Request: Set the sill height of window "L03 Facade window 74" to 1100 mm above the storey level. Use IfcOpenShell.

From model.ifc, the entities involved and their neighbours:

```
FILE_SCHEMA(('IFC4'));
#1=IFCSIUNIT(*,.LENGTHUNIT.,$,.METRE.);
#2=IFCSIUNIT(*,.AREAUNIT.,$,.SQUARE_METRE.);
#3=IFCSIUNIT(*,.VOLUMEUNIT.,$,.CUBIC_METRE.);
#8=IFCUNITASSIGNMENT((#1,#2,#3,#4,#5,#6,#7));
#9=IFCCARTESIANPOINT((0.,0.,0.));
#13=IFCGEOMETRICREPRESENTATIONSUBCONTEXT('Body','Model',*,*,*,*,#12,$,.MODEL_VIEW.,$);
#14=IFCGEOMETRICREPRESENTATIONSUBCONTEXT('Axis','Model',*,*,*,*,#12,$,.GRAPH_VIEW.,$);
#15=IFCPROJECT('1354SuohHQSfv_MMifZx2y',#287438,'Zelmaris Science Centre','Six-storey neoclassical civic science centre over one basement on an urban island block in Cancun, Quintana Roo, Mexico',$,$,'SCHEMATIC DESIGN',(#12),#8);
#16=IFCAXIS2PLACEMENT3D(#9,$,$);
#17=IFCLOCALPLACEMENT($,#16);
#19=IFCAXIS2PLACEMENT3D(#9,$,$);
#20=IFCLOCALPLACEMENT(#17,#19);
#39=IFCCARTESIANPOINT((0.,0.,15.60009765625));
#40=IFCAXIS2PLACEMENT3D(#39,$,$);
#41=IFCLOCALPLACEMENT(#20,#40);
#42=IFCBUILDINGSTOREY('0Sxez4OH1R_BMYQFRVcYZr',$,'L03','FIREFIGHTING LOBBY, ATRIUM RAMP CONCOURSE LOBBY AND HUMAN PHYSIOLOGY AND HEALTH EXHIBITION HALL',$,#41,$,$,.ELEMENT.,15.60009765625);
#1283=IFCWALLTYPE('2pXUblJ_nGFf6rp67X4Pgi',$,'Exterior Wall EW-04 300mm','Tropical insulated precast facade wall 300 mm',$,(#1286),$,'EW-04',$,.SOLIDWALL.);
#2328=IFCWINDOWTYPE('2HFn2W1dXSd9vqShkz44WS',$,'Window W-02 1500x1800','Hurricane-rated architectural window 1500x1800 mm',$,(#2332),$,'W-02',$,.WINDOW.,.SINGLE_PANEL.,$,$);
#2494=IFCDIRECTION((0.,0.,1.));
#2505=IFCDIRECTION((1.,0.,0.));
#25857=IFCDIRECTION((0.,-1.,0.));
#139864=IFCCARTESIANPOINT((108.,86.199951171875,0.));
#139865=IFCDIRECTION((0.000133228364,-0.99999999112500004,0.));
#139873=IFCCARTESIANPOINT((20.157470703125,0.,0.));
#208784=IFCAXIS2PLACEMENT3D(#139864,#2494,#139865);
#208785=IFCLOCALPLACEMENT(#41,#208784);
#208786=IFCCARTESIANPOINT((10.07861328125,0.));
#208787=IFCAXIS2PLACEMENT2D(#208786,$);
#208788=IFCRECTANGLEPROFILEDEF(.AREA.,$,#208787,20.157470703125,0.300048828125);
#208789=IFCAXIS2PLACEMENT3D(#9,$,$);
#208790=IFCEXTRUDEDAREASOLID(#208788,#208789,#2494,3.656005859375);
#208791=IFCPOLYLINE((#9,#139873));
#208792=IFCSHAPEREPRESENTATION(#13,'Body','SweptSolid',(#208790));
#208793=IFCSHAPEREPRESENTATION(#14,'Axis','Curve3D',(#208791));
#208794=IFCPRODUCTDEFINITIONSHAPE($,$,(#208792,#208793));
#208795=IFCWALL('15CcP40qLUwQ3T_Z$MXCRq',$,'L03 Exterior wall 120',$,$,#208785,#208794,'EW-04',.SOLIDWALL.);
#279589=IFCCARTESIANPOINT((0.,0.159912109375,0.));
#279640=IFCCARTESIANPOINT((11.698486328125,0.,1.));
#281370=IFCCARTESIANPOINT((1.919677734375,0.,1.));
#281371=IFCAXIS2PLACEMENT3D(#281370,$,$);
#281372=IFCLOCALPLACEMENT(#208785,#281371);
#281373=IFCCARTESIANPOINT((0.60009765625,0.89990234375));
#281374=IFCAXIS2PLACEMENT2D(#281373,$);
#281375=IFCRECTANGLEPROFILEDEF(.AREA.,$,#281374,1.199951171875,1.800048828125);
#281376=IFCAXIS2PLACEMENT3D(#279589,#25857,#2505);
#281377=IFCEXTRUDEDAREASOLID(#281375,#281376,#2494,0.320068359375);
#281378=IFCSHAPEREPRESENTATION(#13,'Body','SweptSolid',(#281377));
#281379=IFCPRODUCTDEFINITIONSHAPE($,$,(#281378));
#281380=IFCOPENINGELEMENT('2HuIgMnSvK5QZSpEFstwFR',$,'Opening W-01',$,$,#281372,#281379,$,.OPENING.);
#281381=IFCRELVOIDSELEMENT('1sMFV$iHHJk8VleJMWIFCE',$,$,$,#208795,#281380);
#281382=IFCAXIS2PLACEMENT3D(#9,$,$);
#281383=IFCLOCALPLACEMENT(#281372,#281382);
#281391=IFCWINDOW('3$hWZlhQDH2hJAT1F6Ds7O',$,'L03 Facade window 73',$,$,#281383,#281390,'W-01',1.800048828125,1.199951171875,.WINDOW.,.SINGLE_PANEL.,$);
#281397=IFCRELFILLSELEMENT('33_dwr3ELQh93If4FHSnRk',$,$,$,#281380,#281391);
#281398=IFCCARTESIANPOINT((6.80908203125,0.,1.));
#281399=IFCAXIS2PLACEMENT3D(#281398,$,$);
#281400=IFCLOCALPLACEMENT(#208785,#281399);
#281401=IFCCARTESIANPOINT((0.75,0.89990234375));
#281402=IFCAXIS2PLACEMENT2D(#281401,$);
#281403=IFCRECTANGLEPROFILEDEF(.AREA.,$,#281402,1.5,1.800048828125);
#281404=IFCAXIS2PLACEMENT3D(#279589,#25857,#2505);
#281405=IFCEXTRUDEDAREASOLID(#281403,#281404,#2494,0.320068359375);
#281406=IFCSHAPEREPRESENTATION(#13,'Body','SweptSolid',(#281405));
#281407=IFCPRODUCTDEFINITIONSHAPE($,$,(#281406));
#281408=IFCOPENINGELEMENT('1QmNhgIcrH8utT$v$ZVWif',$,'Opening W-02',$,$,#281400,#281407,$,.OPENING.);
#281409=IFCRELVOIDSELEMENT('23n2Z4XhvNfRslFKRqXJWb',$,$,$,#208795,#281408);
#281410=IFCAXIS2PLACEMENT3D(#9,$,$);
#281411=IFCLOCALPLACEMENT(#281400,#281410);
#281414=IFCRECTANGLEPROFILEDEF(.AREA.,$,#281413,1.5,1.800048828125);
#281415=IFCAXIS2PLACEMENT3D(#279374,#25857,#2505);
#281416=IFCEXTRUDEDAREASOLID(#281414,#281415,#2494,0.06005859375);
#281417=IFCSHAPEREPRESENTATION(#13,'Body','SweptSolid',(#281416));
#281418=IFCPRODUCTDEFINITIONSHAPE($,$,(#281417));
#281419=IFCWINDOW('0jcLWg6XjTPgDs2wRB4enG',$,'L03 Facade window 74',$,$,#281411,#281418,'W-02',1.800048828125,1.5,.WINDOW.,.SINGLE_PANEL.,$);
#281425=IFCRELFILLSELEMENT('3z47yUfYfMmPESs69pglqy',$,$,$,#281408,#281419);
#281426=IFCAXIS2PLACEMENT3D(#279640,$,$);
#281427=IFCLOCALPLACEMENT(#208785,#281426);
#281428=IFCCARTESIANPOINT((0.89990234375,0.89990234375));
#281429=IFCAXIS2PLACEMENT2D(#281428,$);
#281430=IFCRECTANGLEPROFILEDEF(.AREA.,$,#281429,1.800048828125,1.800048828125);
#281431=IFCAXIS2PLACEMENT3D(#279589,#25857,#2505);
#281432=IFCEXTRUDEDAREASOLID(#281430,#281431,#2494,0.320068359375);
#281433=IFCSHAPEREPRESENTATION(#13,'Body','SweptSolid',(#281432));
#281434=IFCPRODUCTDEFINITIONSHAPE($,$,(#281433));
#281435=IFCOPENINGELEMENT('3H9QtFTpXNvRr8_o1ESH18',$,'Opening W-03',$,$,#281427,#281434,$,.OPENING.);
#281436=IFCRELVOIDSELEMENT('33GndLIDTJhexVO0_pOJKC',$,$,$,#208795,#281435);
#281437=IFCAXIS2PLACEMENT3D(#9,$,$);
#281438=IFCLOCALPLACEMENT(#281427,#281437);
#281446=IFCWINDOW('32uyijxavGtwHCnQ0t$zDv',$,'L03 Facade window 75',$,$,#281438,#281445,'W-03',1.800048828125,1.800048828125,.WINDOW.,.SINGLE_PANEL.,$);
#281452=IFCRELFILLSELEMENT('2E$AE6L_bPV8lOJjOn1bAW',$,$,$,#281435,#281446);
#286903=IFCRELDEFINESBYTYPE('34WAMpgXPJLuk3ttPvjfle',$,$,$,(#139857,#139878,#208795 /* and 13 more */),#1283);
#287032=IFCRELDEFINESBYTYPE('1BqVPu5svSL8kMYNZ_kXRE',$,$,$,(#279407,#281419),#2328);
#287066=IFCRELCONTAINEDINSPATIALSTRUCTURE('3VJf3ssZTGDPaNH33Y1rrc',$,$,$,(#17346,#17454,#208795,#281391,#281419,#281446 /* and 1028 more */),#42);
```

```python
import numpy as np
import ifcopenshell
import ifcopenshell.api.geometry
import ifcopenshell.geom
import ifcopenshell.util.element
import ifcopenshell.util.placement
import ifcopenshell.util.shape
import ifcopenshell.util.unit

model = ifcopenshell.open("model.ifc")
unit_scale = ifcopenshell.util.unit.calculate_unit_scale(model)

window = model.by_guid("0jcLWg6XjTPgDs2wRB4enG")
opening = window.FillsVoids[0].RelatingOpeningElement
storey = ifcopenshell.util.element.get_container(window, ifc_class="IfcBuildingStorey")
level = ifcopenshell.util.placement.get_local_placement(storey.ObjectPlacement)[2, 3]

# The opening's origin need not be at the sill, so measure its lowest point.
shape = ifcopenshell.geom.create_shape(ifcopenshell.geom.settings(), opening)
bottom = ifcopenshell.util.shape.get_shape_bottom_elevation(shape, shape.geometry) / unit_scale
dz = level + 1.1 - bottom

shift = np.array([0.0, 0.0, dz])
# The window is placed relative to its opening, so it follows when the opening moves.
matrix = ifcopenshell.util.placement.get_local_placement(opening.ObjectPlacement)
matrix[:3, 3] += shift
ifcopenshell.api.geometry.edit_object_placement(
    model, product=opening, matrix=matrix, is_si=False, should_transform_children=True
)

print(f"moved by {dz * unit_scale:+.3f} m")

model.write("model_rev.ifc")
```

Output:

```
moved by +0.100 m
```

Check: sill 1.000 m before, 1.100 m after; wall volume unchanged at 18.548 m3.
